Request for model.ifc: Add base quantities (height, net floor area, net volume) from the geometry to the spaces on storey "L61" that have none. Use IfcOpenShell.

First a look at what the model holds.

```python
import ifcopenshell
import ifcopenshell.util.element
import ifcopenshell.util.unit

model = ifcopenshell.open("model.ifc")
print(model.schema)
for unit_type in ("LENGTHUNIT", "AREAUNIT", "VOLUMEUNIT"):
    print(unit_type, ifcopenshell.util.unit.calculate_unit_scale(model, unit_type))
storey = next(s for s in model.by_type("IfcBuildingStorey") if s.Name == "L61")
spaces = [e for e in ifcopenshell.util.element.get_decomposition(storey) if e.is_a("IfcSpace")]
for e in sorted(spaces, key=lambda e: e.id()):
    print(e.id(), e.is_a(), e.Name, list(ifcopenshell.util.element.get_psets(e, qtos_only=True)), sep=" | ")
```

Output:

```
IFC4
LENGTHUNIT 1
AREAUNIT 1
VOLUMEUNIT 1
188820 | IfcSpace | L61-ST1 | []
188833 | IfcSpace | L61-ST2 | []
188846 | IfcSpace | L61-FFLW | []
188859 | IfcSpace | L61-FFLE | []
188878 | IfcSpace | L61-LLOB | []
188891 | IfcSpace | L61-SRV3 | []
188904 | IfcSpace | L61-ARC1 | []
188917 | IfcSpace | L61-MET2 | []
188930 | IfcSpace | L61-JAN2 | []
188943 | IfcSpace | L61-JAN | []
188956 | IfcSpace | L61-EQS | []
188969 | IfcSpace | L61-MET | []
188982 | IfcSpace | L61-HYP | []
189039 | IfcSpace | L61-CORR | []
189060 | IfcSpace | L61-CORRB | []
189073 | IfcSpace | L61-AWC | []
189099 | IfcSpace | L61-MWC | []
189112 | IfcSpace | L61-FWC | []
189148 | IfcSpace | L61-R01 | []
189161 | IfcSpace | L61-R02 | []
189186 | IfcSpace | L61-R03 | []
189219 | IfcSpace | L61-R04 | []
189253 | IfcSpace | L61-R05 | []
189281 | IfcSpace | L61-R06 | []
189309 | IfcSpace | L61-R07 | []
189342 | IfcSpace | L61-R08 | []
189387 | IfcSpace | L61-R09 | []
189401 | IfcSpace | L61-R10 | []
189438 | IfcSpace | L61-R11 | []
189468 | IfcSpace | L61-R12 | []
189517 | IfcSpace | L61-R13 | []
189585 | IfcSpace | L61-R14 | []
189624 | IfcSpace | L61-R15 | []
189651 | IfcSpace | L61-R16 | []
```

```python
import ifcopenshell
import ifcopenshell.api.pset
import ifcopenshell.geom
import ifcopenshell.util.element
import ifcopenshell.util.shape
import ifcopenshell.util.unit

model = ifcopenshell.open("model.ifc")
unit_scale = ifcopenshell.util.unit.calculate_unit_scale(model)
area_scale = ifcopenshell.util.unit.calculate_unit_scale(model, "AREAUNIT")
volume_scale = ifcopenshell.util.unit.calculate_unit_scale(model, "VOLUMEUNIT")
settings = ifcopenshell.geom.settings()

storey = next(s for s in model.by_type("IfcBuildingStorey") if s.Name == "L61")
spaces = [e for e in ifcopenshell.util.element.get_decomposition(storey) if e.is_a("IfcSpace")]

for e in sorted(spaces, key=lambda e: e.id()):
    if ifcopenshell.util.element.get_psets(e, qtos_only=True, should_inherit=False):
        continue
    # Geometry comes back in metres, in the element's own axes.
    shape = ifcopenshell.geom.create_shape(settings, e)
    values = {
        "Height": ifcopenshell.util.shape.get_z(shape.geometry) / unit_scale,
        "NetFloorArea": ifcopenshell.util.shape.get_footprint_area(shape.geometry) / area_scale,
        "NetVolume": ifcopenshell.util.shape.get_volume(shape.geometry) / volume_scale,
    }
    qto = ifcopenshell.api.pset.add_qto(model, product=e, name="Qto_SpaceBaseQuantities")
    ifcopenshell.api.pset.edit_qto(model, qto=qto, properties=values)
    print(e.id(), {k: round(v, 3) for k, v in values.items()})

model.write("model_edited.ifc")
```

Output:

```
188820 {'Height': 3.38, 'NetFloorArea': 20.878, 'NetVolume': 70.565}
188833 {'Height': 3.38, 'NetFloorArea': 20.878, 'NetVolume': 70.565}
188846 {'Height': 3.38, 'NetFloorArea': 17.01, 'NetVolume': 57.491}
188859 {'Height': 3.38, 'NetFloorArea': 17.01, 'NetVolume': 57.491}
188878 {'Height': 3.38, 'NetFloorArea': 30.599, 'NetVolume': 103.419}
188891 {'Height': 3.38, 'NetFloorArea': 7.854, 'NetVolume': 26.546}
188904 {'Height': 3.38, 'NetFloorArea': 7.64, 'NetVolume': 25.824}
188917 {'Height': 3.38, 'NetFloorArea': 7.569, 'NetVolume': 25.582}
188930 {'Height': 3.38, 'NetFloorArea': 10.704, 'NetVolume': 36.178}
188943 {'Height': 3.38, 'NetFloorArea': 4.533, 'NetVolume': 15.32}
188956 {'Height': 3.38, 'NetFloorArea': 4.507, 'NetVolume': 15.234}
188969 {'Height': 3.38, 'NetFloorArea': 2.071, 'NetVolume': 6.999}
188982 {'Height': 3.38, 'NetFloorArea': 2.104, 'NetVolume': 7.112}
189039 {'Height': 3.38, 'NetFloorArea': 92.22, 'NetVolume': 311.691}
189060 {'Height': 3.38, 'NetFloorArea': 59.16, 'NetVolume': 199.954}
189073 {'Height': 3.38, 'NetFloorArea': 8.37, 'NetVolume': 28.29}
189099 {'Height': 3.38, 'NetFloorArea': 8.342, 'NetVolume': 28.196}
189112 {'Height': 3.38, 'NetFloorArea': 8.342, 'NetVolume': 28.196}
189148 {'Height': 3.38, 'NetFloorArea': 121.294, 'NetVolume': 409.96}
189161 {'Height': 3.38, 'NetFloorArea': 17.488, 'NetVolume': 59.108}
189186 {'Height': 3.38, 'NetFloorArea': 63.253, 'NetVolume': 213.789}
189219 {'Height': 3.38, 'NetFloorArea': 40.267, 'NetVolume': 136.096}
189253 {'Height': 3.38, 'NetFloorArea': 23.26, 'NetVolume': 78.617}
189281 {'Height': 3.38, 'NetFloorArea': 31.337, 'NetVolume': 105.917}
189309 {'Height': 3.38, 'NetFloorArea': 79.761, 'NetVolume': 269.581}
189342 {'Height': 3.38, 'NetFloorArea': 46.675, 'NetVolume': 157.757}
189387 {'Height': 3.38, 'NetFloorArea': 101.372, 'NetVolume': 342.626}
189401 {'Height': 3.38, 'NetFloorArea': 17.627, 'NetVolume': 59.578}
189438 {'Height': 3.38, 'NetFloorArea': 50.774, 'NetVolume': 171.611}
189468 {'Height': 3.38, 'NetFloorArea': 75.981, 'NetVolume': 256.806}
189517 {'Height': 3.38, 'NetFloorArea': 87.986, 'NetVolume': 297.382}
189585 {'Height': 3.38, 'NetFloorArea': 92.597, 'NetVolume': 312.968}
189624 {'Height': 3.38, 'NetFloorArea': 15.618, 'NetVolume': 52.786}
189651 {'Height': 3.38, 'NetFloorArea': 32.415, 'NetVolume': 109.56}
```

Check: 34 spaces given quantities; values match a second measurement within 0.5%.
